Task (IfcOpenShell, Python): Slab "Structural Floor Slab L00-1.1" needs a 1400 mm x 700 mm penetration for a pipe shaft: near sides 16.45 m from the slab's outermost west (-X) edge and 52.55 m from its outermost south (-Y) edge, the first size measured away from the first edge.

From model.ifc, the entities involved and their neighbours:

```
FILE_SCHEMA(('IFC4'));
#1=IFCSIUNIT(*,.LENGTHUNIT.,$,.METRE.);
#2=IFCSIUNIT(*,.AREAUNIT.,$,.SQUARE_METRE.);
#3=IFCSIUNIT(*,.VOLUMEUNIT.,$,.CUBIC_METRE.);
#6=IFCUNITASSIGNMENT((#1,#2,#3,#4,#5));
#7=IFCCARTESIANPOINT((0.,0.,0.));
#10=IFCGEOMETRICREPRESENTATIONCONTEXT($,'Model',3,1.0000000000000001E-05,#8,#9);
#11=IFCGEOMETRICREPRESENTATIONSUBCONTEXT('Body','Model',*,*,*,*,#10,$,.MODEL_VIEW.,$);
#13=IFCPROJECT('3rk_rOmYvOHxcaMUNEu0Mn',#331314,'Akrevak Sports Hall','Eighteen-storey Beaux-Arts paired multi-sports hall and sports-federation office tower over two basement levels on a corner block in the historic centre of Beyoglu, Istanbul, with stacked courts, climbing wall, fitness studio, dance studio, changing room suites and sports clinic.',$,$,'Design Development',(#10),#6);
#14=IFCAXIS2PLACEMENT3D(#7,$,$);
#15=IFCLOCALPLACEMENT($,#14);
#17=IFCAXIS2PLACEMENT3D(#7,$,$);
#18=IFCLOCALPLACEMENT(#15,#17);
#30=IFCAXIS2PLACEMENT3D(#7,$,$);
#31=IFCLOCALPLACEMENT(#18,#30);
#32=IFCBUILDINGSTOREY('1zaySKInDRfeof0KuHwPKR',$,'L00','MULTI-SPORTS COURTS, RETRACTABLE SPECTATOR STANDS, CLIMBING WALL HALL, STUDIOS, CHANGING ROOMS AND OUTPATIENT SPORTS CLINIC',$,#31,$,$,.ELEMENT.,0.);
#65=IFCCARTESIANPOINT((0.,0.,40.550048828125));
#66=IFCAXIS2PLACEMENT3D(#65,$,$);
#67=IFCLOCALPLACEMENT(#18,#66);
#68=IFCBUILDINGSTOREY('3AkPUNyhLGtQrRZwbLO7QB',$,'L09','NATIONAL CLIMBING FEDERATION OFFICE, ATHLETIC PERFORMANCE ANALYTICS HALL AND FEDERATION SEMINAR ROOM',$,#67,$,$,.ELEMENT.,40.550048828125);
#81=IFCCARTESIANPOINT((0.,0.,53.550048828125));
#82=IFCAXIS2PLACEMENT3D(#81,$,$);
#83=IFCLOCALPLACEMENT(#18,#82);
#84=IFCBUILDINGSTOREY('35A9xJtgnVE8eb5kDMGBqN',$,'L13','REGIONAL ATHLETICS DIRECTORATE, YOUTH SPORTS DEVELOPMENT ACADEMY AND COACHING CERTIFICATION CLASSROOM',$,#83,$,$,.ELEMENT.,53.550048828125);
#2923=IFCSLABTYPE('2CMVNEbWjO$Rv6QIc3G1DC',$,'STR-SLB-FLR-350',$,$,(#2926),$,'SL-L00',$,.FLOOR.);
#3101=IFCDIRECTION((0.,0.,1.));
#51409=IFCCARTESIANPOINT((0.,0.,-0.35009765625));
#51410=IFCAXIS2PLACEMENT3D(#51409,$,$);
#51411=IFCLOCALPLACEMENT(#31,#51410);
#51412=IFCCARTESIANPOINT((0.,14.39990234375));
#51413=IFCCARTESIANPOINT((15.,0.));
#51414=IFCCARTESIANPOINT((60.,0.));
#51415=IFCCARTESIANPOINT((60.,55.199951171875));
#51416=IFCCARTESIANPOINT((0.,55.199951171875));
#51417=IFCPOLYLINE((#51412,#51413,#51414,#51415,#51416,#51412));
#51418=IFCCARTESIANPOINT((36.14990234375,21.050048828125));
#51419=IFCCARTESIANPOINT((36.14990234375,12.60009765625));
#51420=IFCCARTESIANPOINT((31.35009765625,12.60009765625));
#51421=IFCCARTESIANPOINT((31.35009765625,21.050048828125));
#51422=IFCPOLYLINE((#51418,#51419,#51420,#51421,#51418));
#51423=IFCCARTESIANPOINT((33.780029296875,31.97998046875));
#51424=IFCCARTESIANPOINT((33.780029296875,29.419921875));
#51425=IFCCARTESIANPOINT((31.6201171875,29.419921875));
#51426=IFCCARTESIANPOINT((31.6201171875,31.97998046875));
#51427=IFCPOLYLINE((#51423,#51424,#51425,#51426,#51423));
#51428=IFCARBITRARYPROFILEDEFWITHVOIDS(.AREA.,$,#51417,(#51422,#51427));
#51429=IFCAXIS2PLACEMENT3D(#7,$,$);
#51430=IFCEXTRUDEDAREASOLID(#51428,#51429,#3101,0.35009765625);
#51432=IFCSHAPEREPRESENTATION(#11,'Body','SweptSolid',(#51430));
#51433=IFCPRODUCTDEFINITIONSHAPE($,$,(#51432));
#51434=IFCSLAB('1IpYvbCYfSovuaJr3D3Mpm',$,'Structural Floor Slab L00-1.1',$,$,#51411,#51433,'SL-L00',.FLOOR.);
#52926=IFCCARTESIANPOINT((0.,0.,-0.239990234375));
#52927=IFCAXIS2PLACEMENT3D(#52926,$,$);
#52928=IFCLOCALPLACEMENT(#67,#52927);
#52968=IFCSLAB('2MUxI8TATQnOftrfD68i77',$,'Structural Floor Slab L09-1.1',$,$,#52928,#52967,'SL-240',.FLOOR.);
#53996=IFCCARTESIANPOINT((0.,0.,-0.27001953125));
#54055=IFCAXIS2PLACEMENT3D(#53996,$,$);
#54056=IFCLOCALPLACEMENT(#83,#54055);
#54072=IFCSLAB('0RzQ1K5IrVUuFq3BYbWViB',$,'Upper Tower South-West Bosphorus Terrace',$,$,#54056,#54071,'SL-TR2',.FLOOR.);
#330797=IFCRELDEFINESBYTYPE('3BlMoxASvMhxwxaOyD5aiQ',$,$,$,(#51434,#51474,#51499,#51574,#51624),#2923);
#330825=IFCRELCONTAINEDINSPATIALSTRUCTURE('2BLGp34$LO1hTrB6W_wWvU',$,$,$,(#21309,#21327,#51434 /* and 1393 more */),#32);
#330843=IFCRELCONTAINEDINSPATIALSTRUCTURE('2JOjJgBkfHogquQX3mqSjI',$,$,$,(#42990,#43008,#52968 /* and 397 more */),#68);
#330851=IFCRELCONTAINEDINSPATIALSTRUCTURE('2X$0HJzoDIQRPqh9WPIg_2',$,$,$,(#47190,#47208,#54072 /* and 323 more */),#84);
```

```python
import numpy as np
import ifcopenshell
import ifcopenshell.api.feature
import ifcopenshell.api.geometry
import ifcopenshell.api.root
import ifcopenshell.geom
import ifcopenshell.util.placement
import ifcopenshell.util.representation
import ifcopenshell.util.shape
import ifcopenshell.util.unit

model = ifcopenshell.open("model.ifc")
unit_scale = ifcopenshell.util.unit.calculate_unit_scale(model)
settings = ifcopenshell.geom.settings()


def volume(element):
    """Net volume in cubic metres, openings subtracted."""
    shape = ifcopenshell.geom.create_shape(settings, element)
    return ifcopenshell.util.shape.get_volume(shape.geometry)


slab = model.by_guid("1IpYvbCYfSovuaJr3D3Mpm")
before = volume(slab)

# Extent in the slab's own axes, in metres. The edges named are its -X and -Y sides.
slab_shape = ifcopenshell.geom.create_shape(settings, slab)
vertices = ifcopenshell.util.shape.get_vertices(slab_shape.geometry)
x_min, y_min, bottom = vertices.min(axis=0)
top = vertices[:, 2].max()

opening = ifcopenshell.api.root.create_entity(model, ifc_class="IfcOpeningElement", name="Pipe shaft opening", predefined_type="OPENING")
context = ifcopenshell.util.representation.get_context(model, "Model", "Body", "MODEL_VIEW")
width, depth = 1.4, 0.7
outline = [(0.0, 0.0), (width, 0.0), (width, depth), (0.0, depth), (0.0, 0.0)]
# Overshoot both faces by 50 mm so the cut is clean.
shape = ifcopenshell.api.geometry.add_slab_representation(
    model, context=context, depth=top - bottom + 0.1, polyline=outline
)
ifcopenshell.api.geometry.assign_representation(model, product=opening, representation=shape)

matrix = ifcopenshell.util.placement.get_local_placement(slab.ObjectPlacement)
matrix[:, 3] = matrix @ np.append(np.array([x_min + 16.45, y_min + 52.55, bottom - 0.05]) / unit_scale, 1.0)
ifcopenshell.api.geometry.edit_object_placement(model, product=opening, matrix=matrix, is_si=False)
ifcopenshell.api.feature.add_feature(model, feature=opening, element=slab)

after = volume(slab)

print(f"slab volume {before:.3f} -> {after:.3f} m3")

model.write("model_updated.ifc")
```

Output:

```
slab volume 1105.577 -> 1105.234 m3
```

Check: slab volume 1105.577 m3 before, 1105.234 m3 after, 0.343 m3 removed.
